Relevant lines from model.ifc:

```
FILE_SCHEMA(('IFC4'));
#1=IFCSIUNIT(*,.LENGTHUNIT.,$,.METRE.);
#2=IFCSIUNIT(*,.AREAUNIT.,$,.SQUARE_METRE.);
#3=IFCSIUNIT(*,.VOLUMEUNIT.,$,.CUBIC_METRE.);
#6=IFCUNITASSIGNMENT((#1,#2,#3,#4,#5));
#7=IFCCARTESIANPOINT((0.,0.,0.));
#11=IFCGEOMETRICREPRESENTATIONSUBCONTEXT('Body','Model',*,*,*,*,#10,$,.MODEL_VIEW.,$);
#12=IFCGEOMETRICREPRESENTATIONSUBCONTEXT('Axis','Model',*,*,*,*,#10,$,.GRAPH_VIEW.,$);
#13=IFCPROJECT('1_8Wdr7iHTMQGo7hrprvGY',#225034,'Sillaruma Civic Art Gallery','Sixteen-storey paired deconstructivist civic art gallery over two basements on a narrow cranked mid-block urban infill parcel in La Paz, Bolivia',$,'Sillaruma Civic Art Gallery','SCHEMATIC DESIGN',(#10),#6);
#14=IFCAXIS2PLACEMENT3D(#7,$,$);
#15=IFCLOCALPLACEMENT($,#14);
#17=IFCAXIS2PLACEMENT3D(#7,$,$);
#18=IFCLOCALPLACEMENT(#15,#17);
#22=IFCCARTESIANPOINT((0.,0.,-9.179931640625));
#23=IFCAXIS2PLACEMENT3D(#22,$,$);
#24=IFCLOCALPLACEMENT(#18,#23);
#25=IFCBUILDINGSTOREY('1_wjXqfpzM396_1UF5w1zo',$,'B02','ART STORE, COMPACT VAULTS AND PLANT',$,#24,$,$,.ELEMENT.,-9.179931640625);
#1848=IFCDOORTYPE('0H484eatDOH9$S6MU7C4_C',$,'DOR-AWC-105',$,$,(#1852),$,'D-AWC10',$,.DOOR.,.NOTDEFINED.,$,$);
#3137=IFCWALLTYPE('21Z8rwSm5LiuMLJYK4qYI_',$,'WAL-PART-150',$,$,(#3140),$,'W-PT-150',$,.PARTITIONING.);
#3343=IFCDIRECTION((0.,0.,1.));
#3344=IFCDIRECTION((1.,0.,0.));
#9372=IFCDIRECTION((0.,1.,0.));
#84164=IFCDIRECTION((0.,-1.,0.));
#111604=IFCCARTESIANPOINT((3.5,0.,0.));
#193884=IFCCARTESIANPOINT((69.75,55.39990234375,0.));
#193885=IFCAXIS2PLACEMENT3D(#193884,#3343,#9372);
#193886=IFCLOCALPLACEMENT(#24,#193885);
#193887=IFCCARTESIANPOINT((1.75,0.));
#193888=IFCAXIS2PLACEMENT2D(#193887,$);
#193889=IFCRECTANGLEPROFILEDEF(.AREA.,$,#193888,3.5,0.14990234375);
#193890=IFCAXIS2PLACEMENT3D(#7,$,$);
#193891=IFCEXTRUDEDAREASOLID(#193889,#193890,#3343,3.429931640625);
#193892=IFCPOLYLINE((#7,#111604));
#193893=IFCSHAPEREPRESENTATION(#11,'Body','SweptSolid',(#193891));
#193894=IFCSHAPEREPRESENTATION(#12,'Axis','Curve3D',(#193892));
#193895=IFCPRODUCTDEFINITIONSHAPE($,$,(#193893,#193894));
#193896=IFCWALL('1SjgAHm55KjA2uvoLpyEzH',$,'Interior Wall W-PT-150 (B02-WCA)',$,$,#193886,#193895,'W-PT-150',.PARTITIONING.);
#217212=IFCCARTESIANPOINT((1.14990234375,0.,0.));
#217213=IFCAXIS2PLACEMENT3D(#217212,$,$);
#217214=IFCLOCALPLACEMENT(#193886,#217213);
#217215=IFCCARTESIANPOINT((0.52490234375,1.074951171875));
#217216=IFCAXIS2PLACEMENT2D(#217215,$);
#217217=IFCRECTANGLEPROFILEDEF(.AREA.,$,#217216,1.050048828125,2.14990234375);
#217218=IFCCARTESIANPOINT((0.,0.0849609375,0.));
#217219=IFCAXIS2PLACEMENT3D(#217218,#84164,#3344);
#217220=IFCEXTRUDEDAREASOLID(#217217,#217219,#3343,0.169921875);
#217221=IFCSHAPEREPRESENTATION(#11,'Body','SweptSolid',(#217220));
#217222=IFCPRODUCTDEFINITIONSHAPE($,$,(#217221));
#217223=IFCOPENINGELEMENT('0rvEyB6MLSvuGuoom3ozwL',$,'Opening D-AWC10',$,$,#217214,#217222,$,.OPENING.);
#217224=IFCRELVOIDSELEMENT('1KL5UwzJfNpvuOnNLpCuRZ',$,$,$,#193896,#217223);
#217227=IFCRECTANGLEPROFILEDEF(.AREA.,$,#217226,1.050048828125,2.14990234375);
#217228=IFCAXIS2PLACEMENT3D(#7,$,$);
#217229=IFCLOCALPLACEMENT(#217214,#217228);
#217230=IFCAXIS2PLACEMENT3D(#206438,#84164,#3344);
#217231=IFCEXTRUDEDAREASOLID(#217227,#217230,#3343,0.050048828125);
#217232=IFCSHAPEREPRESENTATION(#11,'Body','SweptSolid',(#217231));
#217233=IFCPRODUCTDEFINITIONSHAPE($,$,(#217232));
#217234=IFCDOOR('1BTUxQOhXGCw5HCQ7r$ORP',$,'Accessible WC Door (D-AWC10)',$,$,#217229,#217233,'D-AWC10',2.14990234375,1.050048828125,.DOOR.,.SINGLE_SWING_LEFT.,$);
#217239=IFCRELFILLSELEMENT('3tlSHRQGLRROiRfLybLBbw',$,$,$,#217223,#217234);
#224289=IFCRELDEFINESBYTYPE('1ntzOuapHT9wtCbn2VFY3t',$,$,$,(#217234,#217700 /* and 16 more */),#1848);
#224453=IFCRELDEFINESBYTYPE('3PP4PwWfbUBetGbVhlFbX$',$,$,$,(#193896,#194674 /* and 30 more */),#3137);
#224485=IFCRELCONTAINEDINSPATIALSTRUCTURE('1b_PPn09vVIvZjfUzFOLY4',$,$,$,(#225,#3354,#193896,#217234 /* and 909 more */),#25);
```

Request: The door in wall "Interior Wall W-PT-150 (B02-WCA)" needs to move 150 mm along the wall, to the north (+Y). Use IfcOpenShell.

```python
import ifcopenshell
import ifcopenshell.api.geometry
import ifcopenshell.util.placement

model = ifcopenshell.open("model.ifc")

door = model.by_id(217234)
opening = door.FillsVoids[0].RelatingOpeningElement
wall = opening.VoidsElements[0].RelatingBuildingElement

wall_matrix = ifcopenshell.util.placement.get_local_placement(wall.ObjectPlacement)
shift = wall_matrix[:3, 0] * 0.15
before = ifcopenshell.util.placement.get_local_placement(door.ObjectPlacement)[:3, 3].copy()

# The door is placed relative to its opening, so it follows when the opening moves.
matrix = ifcopenshell.util.placement.get_local_placement(opening.ObjectPlacement)
matrix[:3, 3] += shift
ifcopenshell.api.geometry.edit_object_placement(
    model, product=opening, matrix=matrix, is_si=False, should_transform_children=True
)

after = ifcopenshell.util.placement.get_local_placement(door.ObjectPlacement)[:3, 3]
print("door moved by", (after - before).round(3) + 0.0)

model.write("model_updated.ifc")
```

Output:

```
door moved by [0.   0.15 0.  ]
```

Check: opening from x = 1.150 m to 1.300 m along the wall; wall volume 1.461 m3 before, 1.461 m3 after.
